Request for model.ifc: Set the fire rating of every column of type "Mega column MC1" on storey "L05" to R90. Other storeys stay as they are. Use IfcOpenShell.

First a look at what the model holds.

```python
import ifcopenshell
import ifcopenshell.util.element

model = ifcopenshell.open("model.ifc")
print(model.schema)
storey = next(s for s in model.by_type("IfcBuildingStorey") if s.Name == "L05")
columns = [e for e in ifcopenshell.util.element.get_decomposition(storey) if e.is_a("IfcColumn")]
seen = {}
for e in columns:
    element_type = ifcopenshell.util.element.get_type(e)
    key = (element_type.Name if element_type != e and element_type else None, ifcopenshell.util.element.get_pset(e, "Pset_ColumnCommon", "FireRating"))
    seen[key] = seen.get(key, 0) + 1
for (name, value), count in sorted(seen.items(), key=str):
    print(count, "x", name, "|", value)
```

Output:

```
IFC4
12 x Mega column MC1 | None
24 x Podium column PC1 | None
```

```python
import ifcopenshell
import ifcopenshell.api.pset
import ifcopenshell.util.element

model = ifcopenshell.open("model.ifc")

storey = next(s for s in model.by_type("IfcBuildingStorey") if s.Name == "L05")
columns = [e for e in ifcopenshell.util.element.get_decomposition(storey) if e.is_a("IfcColumn")]

count = 0
for e in columns:
    element_type = ifcopenshell.util.element.get_type(e)
    if element_type in (None, e) or element_type.Name != "Mega column MC1":
        continue
    found = ifcopenshell.util.element.get_pset(e, "Pset_ColumnCommon", should_inherit=False)
    if found:
        pset = model.by_id(found["id"])
        if len(ifcopenshell.util.element.get_elements_by_pset(pset)) > 1:
            pset = ifcopenshell.api.pset.unshare_pset(model, products=[e], pset=pset)[0]
    else:
        pset = ifcopenshell.api.pset.add_pset(model, product=e, name="Pset_ColumnCommon")
    ifcopenshell.api.pset.edit_pset(model, pset=pset, properties={"FireRating": "R90"})
    count += 1

print(count, "columns updated")

model.write("model_updated.ifc")
```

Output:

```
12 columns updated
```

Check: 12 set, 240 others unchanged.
